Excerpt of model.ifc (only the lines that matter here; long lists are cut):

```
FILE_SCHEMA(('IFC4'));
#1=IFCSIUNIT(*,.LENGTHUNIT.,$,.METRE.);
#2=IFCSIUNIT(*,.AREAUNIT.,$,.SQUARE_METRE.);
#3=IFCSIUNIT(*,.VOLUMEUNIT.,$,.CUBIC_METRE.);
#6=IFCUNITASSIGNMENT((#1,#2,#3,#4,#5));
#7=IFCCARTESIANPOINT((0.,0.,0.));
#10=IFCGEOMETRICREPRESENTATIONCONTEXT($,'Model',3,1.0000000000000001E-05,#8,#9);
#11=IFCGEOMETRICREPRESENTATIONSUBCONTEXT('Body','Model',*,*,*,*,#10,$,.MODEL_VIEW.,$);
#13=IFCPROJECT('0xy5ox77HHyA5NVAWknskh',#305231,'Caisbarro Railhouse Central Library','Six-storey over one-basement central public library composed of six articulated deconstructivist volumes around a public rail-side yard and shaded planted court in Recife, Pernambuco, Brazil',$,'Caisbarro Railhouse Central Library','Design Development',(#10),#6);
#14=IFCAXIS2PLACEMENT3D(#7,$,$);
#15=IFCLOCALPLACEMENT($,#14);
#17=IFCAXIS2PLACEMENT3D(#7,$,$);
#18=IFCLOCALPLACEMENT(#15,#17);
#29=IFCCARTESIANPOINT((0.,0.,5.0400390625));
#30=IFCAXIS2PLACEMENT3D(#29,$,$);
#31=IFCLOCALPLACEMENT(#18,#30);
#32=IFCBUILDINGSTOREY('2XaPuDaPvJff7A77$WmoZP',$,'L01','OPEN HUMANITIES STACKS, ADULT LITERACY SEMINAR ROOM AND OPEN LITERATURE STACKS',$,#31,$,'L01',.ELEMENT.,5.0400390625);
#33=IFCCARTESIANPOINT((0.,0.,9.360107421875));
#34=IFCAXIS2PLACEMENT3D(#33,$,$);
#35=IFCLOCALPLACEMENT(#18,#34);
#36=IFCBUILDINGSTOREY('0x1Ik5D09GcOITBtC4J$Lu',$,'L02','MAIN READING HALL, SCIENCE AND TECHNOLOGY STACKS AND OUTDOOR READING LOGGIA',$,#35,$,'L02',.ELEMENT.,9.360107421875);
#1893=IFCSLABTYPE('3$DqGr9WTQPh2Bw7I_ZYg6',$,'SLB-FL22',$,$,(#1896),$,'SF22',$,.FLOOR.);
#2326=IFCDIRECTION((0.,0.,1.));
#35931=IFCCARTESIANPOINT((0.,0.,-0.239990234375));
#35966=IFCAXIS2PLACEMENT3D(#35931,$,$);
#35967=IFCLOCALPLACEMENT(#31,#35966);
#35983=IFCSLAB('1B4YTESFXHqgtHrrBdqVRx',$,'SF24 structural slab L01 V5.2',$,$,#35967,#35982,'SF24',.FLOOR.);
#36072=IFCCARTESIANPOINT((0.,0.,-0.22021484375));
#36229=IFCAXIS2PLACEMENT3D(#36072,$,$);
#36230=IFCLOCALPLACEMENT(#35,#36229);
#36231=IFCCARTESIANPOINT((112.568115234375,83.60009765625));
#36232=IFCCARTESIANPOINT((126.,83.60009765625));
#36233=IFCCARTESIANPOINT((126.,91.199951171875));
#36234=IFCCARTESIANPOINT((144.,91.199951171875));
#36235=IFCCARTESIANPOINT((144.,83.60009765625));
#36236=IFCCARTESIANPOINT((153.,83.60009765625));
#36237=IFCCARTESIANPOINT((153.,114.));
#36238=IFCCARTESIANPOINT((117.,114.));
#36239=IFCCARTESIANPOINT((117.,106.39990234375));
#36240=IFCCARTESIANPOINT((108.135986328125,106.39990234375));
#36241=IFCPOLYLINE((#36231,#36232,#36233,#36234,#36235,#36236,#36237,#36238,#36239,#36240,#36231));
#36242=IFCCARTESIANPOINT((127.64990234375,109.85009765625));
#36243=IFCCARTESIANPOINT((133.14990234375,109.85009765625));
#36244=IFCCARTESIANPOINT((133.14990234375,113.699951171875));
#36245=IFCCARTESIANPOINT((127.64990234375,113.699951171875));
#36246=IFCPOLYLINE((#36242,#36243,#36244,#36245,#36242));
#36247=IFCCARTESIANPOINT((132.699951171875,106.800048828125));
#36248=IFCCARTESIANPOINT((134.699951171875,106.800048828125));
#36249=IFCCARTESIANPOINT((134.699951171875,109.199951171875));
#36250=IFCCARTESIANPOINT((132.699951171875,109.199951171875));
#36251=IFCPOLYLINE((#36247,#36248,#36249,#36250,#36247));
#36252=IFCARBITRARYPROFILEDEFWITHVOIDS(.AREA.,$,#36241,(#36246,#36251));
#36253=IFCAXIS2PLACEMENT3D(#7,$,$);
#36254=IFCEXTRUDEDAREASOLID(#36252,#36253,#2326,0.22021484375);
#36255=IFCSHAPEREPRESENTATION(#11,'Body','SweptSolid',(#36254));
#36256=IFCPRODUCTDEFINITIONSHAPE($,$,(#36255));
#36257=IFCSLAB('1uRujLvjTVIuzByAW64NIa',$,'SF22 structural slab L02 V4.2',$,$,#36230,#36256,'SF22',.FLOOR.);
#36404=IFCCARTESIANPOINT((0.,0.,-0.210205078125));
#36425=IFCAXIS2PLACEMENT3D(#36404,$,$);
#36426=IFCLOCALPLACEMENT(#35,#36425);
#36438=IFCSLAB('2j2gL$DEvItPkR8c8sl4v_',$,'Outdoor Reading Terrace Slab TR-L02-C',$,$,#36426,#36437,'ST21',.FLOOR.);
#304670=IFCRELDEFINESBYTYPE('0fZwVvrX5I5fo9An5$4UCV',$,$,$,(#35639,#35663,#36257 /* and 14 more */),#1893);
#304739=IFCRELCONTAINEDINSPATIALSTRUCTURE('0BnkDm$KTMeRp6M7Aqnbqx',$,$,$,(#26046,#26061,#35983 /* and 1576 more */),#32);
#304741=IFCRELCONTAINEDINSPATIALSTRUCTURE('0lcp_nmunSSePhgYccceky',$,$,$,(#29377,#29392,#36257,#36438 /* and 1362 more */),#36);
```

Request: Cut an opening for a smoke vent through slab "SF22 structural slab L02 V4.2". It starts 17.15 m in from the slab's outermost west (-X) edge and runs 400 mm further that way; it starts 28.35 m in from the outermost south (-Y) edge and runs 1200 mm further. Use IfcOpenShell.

```python
import numpy as np
import ifcopenshell
import ifcopenshell.api.feature
import ifcopenshell.api.geometry
import ifcopenshell.api.root
import ifcopenshell.geom
import ifcopenshell.util.placement
import ifcopenshell.util.representation
import ifcopenshell.util.shape
import ifcopenshell.util.unit

model = ifcopenshell.open("model.ifc")
unit_scale = ifcopenshell.util.unit.calculate_unit_scale(model)
settings = ifcopenshell.geom.settings()


def volume(element):
    """Net volume in cubic metres, openings subtracted."""
    shape = ifcopenshell.geom.create_shape(settings, element)
    return ifcopenshell.util.shape.get_volume(shape.geometry)


slab = model.by_guid("1uRujLvjTVIuzByAW64NIa")
before = volume(slab)

# Extent in the slab's own axes, in metres. The edges named are its -X and -Y sides.
slab_shape = ifcopenshell.geom.create_shape(settings, slab)
vertices = ifcopenshell.util.shape.get_vertices(slab_shape.geometry)
x_min, y_min, bottom = vertices.min(axis=0)
top = vertices[:, 2].max()

opening = ifcopenshell.api.root.create_entity(model, ifc_class="IfcOpeningElement", name="Smoke vent opening", predefined_type="OPENING")
context = ifcopenshell.util.representation.get_context(model, "Model", "Body", "MODEL_VIEW")
width, depth = 0.4, 1.2
outline = [(0.0, 0.0), (width, 0.0), (width, depth), (0.0, depth), (0.0, 0.0)]
# Overshoot both faces by 50 mm so the cut is clean.
shape = ifcopenshell.api.geometry.add_slab_representation(
    model, context=context, depth=top - bottom + 0.1, polyline=outline
)
ifcopenshell.api.geometry.assign_representation(model, product=opening, representation=shape)

matrix = ifcopenshell.util.placement.get_local_placement(slab.ObjectPlacement)
matrix[:, 3] = matrix @ np.append(np.array([x_min + 17.15, y_min + 28.35, bottom - 0.05]) / unit_scale, 1.0)
ifcopenshell.api.geometry.edit_object_placement(model, product=opening, matrix=matrix, is_si=False)
ifcopenshell.api.feature.add_feature(model, feature=opening, element=slab)

after = volume(slab)

print(f"slab volume {before:.3f} -> {after:.3f} m3")

model.write("model_rev.ifc")
```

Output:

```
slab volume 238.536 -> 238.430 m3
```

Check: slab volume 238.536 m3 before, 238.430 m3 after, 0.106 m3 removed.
